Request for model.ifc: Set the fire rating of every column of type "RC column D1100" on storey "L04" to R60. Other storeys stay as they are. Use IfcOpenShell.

First a look at what the model holds.

```python
import ifcopenshell
import ifcopenshell.util.element

model = ifcopenshell.open("model.ifc")
print(model.schema)
storey = next(s for s in model.by_type("IfcBuildingStorey") if s.Name == "L04")
columns = [e for e in ifcopenshell.util.element.get_decomposition(storey) if e.is_a("IfcColumn")]
seen = {}
for e in columns:
    element_type = ifcopenshell.util.element.get_type(e)
    key = (element_type.Name if element_type != e and element_type else None, ifcopenshell.util.element.get_pset(e, "Pset_ColumnCommon", "FireRating"))
    seen[key] = seen.get(key, 0) + 1
for (name, value), count in sorted(seen.items(), key=str):
    print(count, "x", name, "|", value)
```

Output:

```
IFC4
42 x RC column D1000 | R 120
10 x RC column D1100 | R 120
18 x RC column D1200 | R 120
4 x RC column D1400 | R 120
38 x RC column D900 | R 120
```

```python
import ifcopenshell
import ifcopenshell.api.pset
import ifcopenshell.util.element

model = ifcopenshell.open("model.ifc")

storey = next(s for s in model.by_type("IfcBuildingStorey") if s.Name == "L04")
columns = [e for e in ifcopenshell.util.element.get_decomposition(storey) if e.is_a("IfcColumn")]

count = 0
for e in columns:
    element_type = ifcopenshell.util.element.get_type(e)
    if element_type in (None, e) or element_type.Name != "RC column D1100":
        continue
    # add_pset returns the element's existing set when there is one.
    pset = ifcopenshell.api.pset.add_pset(model, product=e, name="Pset_ColumnCommon")
    ifcopenshell.api.pset.edit_pset(model, pset=pset, properties={"FireRating": "R60"})
    count += 1

print(count, "columns updated")

model.write("model_v2.ifc")
```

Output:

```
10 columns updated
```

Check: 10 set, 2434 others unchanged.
